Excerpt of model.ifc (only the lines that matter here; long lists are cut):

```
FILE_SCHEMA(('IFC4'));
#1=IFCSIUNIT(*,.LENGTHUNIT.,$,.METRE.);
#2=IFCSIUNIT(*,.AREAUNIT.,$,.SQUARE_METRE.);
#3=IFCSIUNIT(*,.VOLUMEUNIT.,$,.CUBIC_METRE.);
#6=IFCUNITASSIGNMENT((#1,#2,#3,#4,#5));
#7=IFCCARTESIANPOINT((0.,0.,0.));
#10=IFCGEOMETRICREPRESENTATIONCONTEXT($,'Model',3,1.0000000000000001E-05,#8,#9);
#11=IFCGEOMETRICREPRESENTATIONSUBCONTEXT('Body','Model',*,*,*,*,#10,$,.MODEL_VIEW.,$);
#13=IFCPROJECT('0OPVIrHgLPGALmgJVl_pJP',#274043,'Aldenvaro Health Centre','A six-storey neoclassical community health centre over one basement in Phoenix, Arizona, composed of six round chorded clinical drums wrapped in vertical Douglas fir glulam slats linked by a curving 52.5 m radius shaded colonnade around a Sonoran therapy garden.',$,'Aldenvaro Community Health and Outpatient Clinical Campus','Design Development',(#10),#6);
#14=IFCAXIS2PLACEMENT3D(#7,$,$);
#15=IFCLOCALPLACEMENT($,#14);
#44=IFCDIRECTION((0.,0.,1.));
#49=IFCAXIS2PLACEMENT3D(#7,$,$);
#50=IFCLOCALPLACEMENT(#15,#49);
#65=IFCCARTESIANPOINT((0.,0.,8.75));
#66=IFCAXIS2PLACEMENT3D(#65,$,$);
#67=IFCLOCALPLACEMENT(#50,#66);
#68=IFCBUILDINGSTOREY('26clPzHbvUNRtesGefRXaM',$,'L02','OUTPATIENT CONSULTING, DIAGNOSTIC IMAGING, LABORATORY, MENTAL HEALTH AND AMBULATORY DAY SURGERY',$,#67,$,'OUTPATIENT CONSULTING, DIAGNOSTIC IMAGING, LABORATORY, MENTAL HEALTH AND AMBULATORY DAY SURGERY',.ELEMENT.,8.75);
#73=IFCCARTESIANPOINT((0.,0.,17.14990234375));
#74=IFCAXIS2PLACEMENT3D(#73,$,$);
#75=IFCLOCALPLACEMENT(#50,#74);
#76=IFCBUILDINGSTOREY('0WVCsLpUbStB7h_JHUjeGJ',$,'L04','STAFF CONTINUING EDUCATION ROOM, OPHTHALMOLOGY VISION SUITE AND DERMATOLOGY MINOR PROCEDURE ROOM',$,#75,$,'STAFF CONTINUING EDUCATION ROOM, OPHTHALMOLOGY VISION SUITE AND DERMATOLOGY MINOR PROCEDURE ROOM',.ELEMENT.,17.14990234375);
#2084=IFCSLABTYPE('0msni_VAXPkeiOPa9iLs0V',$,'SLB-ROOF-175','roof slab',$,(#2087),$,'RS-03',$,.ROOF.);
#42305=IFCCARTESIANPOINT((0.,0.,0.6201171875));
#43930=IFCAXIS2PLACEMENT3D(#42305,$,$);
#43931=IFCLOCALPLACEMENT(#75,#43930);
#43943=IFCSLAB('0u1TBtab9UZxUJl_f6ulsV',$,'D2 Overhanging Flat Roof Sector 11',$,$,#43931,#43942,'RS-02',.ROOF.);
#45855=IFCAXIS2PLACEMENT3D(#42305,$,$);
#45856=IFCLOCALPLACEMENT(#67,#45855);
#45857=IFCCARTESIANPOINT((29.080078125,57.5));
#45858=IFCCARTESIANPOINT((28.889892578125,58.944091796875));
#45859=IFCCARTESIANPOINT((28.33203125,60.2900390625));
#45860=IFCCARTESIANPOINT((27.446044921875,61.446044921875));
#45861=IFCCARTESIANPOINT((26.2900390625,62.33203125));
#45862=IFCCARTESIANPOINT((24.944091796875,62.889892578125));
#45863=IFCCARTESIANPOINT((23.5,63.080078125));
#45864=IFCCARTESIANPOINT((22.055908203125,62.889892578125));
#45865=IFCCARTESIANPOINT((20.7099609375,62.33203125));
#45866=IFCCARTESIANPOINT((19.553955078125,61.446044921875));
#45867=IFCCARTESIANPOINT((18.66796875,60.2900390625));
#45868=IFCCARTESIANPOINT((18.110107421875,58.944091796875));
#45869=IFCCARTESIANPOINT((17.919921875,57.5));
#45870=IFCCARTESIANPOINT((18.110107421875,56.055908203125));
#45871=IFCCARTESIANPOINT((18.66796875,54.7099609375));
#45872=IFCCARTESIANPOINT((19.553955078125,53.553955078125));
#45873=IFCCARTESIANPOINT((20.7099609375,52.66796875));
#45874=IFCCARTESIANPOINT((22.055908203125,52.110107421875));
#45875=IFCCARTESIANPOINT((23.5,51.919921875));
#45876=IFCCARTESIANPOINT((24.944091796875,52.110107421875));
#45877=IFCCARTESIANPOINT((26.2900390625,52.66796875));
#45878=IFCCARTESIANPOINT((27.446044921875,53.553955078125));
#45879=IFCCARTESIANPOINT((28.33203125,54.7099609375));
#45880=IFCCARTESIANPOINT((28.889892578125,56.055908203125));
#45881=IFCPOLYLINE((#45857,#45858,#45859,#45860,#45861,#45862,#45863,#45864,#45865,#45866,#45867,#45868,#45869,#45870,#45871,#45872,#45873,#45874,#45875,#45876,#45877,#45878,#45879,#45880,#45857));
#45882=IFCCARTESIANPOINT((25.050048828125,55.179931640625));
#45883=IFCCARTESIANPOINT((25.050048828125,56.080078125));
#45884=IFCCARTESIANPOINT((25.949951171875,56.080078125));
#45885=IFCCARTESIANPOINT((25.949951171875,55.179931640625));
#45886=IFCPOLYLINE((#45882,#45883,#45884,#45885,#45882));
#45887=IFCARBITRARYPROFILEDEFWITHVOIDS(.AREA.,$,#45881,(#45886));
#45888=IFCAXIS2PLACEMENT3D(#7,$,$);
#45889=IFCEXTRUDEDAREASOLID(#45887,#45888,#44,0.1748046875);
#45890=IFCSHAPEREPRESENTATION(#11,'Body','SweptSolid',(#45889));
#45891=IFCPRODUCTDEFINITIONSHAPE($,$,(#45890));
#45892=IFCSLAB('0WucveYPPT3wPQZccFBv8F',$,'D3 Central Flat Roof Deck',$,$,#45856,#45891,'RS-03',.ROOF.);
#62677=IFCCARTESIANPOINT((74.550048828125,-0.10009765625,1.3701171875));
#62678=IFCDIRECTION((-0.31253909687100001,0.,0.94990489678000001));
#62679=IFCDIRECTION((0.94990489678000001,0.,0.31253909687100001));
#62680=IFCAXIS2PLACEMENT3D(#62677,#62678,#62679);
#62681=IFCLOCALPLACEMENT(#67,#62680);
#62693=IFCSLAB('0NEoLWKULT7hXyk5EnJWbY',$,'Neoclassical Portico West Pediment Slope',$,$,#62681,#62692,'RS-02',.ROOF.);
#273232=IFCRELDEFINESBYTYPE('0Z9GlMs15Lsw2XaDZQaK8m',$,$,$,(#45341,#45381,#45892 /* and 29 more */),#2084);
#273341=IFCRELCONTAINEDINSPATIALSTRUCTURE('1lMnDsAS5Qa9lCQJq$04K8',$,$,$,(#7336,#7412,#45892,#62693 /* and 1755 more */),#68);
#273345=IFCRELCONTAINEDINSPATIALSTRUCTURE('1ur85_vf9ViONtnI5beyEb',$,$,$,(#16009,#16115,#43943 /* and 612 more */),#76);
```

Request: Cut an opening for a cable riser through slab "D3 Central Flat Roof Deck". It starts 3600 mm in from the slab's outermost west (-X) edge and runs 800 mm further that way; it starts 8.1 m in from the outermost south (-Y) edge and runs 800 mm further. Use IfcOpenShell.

```python
import numpy as np
import ifcopenshell
import ifcopenshell.api.feature
import ifcopenshell.api.geometry
import ifcopenshell.api.root
import ifcopenshell.geom
import ifcopenshell.util.placement
import ifcopenshell.util.representation
import ifcopenshell.util.shape
import ifcopenshell.util.unit

model = ifcopenshell.open("model.ifc")
unit_scale = ifcopenshell.util.unit.calculate_unit_scale(model)
settings = ifcopenshell.geom.settings()


def volume(element):
    """Net volume in cubic metres, openings subtracted."""
    shape = ifcopenshell.geom.create_shape(settings, element)
    return ifcopenshell.util.shape.get_volume(shape.geometry)


slab = model.by_guid("0WucveYPPT3wPQZccFBv8F")
before = volume(slab)

# Extent in the slab's own axes, in metres. The edges named are its -X and -Y sides.
slab_shape = ifcopenshell.geom.create_shape(settings, slab)
vertices = ifcopenshell.util.shape.get_vertices(slab_shape.geometry)
x_min, y_min, bottom = vertices.min(axis=0)
top = vertices[:, 2].max()

opening = ifcopenshell.api.root.create_entity(model, ifc_class="IfcOpeningElement", name="Cable riser opening", predefined_type="OPENING")
context = ifcopenshell.util.representation.get_context(model, "Model", "Body", "MODEL_VIEW")
width, depth = 0.8, 0.8
outline = [(0.0, 0.0), (width, 0.0), (width, depth), (0.0, depth), (0.0, 0.0)]
# Overshoot both faces by 50 mm so the cut is clean.
shape = ifcopenshell.api.geometry.add_slab_representation(
    model, context=context, depth=top - bottom + 0.1, polyline=outline
)
ifcopenshell.api.geometry.assign_representation(model, product=opening, representation=shape)

matrix = ifcopenshell.util.placement.get_local_placement(slab.ObjectPlacement)
matrix[:, 3] = matrix @ np.append(np.array([x_min + 3.6, y_min + 8.1, bottom - 0.05]) / unit_scale, 1.0)
ifcopenshell.api.geometry.edit_object_placement(model, product=opening, matrix=matrix, is_si=False)
ifcopenshell.api.feature.add_feature(model, feature=opening, element=slab)

after = volume(slab)

print(f"slab volume {before:.3f} -> {after:.3f} m3")

model.write("model_rev.ifc")
```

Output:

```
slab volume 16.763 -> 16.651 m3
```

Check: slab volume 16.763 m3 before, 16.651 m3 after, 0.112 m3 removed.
